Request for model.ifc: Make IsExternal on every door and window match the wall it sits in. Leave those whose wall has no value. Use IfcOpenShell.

First a look at what the model holds.

```python
import ifcopenshell
import ifcopenshell.util.element

model = ifcopenshell.open("model.ifc")
print(model.schema)
seen = {}
for e in model.by_type("IfcDoor") + model.by_type("IfcWindow"):
    if not e.FillsVoids:
        continue
    host = e.FillsVoids[0].RelatingOpeningElement.VoidsElements[0].RelatingBuildingElement
    own = ifcopenshell.util.element.get_pset(e, f"Pset_{e.is_a()[3:].removesuffix('StandardCase')}Common", "IsExternal")
    wall = ifcopenshell.util.element.get_pset(host, "Pset_WallCommon", "IsExternal")
    seen[e.is_a(), own, wall] = seen.get((e.is_a(), own, wall), 0) + 1
for (cls, own, wall), count in sorted(seen.items(), key=str):
    print(count, cls, "IsExternal:", own, "| host wall:", wall)
```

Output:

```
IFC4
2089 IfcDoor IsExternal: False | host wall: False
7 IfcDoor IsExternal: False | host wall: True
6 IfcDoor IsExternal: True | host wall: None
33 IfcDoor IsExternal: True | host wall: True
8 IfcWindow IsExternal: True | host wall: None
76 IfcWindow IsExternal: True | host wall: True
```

```python
import ifcopenshell
import ifcopenshell.api.pset
import ifcopenshell.util.element

model = ifcopenshell.open("model.ifc")

count = 0
for ifc_class, pset_name in (("IfcDoor", "Pset_DoorCommon"), ("IfcWindow", "Pset_WindowCommon")):
    for e in model.by_type(ifc_class):
        if not e.FillsVoids:
            continue
        host = e.FillsVoids[0].RelatingOpeningElement.VoidsElements[0].RelatingBuildingElement
        external = ifcopenshell.util.element.get_pset(host, "Pset_WallCommon", "IsExternal")
        if external is None or ifcopenshell.util.element.get_pset(e, pset_name, "IsExternal") == external:
            continue
        found = ifcopenshell.util.element.get_pset(e, pset_name, should_inherit=False)
        if found:
            pset = model.by_id(found["id"])
            if len(ifcopenshell.util.element.get_elements_by_pset(pset)) > 1:
                pset = ifcopenshell.api.pset.unshare_pset(model, products=[e], pset=pset)[0]
        else:
            pset = ifcopenshell.api.pset.add_pset(model, product=e, name=pset_name)
        ifcopenshell.api.pset.edit_pset(model, pset=pset, properties={"IsExternal": external})
        count += 1

print(count, "updated")

model.write("model_rev.ifc")
```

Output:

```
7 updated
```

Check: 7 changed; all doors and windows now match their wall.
